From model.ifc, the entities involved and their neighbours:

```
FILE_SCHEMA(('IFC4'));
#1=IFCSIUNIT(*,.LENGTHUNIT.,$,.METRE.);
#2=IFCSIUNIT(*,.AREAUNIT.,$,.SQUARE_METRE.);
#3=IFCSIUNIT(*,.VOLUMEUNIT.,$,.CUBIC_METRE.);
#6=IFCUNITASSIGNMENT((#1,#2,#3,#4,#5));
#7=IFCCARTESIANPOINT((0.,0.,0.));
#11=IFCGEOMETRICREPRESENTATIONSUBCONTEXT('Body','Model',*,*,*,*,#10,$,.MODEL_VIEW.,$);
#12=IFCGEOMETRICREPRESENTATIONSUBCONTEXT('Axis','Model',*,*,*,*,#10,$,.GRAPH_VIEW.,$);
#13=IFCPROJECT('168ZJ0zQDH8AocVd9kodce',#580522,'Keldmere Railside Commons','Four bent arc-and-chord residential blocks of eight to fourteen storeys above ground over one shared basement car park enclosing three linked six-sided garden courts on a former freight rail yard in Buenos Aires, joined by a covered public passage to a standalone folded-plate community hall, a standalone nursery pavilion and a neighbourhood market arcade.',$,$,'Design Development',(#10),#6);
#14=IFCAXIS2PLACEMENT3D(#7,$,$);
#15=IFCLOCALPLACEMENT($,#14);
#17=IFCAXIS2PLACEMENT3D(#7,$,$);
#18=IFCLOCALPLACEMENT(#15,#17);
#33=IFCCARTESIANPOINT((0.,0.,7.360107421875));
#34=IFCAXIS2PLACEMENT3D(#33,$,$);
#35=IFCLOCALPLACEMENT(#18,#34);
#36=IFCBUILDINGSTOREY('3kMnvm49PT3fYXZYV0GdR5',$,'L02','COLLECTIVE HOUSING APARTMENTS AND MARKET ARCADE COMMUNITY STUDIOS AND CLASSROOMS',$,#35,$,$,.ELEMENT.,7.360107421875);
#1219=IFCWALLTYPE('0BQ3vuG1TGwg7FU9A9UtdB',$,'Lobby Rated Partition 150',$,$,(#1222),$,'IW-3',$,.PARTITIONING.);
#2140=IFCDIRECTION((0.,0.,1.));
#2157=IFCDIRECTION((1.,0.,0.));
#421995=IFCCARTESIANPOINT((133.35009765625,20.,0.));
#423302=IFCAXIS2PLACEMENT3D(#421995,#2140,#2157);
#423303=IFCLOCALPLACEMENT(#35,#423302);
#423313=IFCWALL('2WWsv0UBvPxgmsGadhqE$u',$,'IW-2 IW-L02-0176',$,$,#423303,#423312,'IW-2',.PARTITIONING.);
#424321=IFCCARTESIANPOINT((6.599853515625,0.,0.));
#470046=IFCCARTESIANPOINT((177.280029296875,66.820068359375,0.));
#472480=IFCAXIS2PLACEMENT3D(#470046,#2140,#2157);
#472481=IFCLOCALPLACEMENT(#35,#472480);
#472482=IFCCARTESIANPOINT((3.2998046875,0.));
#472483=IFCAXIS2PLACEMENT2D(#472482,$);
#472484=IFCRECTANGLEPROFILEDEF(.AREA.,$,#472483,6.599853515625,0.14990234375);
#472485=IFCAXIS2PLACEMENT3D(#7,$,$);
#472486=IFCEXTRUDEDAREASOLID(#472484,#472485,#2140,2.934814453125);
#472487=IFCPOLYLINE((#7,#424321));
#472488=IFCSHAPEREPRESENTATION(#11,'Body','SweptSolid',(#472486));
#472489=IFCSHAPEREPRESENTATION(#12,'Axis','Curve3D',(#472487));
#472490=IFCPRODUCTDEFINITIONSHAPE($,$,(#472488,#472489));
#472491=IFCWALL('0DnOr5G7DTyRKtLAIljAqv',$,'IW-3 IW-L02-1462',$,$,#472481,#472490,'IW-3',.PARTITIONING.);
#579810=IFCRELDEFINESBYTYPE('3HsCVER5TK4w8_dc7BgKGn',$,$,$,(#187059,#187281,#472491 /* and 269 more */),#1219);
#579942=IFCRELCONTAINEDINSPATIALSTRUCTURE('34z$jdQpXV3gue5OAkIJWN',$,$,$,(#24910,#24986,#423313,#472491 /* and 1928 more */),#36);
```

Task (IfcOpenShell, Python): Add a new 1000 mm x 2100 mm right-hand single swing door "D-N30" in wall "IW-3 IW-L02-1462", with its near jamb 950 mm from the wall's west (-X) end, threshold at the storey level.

```python
import numpy as np
import ifcopenshell
import ifcopenshell.api.feature
import ifcopenshell.api.geometry
import ifcopenshell.api.root
import ifcopenshell.api.spatial
import ifcopenshell.geom
import ifcopenshell.util.element
import ifcopenshell.util.placement
import ifcopenshell.util.representation
import ifcopenshell.util.shape
import ifcopenshell.util.unit

model = ifcopenshell.open("model.ifc")
unit_scale = ifcopenshell.util.unit.calculate_unit_scale(model)
settings = ifcopenshell.geom.settings()


def volume(element):
    """Net volume in cubic metres, openings subtracted."""
    shape = ifcopenshell.geom.create_shape(settings, element)
    return ifcopenshell.util.shape.get_volume(shape.geometry)


wall = model.by_guid("0DnOr5G7DTyRKtLAIljAqv")
storey = ifcopenshell.util.element.get_container(wall, ifc_class="IfcBuildingStorey")
context = ifcopenshell.util.representation.get_context(model, "Model", "Body", "MODEL_VIEW")
before = volume(wall)

width, height, from_end, sill = 1, 2.1, 0.95, 0.0  # metres

# The wall runs along its own X axis, and the end named is its -X end.
wall_shape = ifcopenshell.geom.create_shape(settings, wall)
x, y, z = ifcopenshell.util.shape.get_vertices(wall_shape.geometry).T
start = x.min() + from_end
face, thickness = float(y.min()), float(y.max() - y.min())
wall_matrix = ifcopenshell.util.placement.get_local_placement(wall.ObjectPlacement)
level = ifcopenshell.util.placement.get_local_placement(storey.ObjectPlacement)[2, 3]


def in_wall(x, y):
    """Placement at x, y metres in the wall's axes, at sill height."""
    matrix = wall_matrix.copy()
    matrix[:, 3] = wall_matrix @ np.array([x / unit_scale, y / unit_scale, 0.0, 1.0])
    matrix[2, 3] = level + sill / unit_scale
    return matrix


# Opening: a box that overshoots both wall faces by 50 mm.
opening = ifcopenshell.api.root.create_entity(model, ifc_class="IfcOpeningElement", predefined_type="OPENING")
box = ifcopenshell.api.geometry.add_wall_representation(
    model, context=context, length=width, height=height, thickness=thickness + 0.1
)
ifcopenshell.api.geometry.assign_representation(model, product=opening, representation=box)
ifcopenshell.api.geometry.edit_object_placement(model, product=opening, matrix=in_wall(start, face - 0.05), is_si=False)
ifcopenshell.api.feature.add_feature(model, feature=opening, element=wall)

door = ifcopenshell.api.root.create_entity(model, ifc_class="IfcDoor", name="D-N30", predefined_type="DOOR")
door.OverallWidth, door.OverallHeight = width / unit_scale, height / unit_scale
door.OperationType = "SINGLE_SWING_RIGHT"
body = ifcopenshell.api.geometry.add_door_representation(
    model,
    context=context,
    overall_width=door.OverallWidth,
    overall_height=door.OverallHeight,
    operation_type="SINGLE_SWING_RIGHT",
    lining_properties={"LiningDepth": thickness / unit_scale, "ThresholdDepth": thickness / unit_scale},
)
ifcopenshell.api.geometry.assign_representation(model, product=door, representation=body)
ifcopenshell.api.spatial.assign_container(model, products=[door], relating_structure=storey)
ifcopenshell.api.feature.add_filling(model, opening=opening, element=door)

# The lining spans the wall, so the door starts at the wall face.
ifcopenshell.api.geometry.edit_object_placement(model, product=door, matrix=in_wall(start, face), is_si=False)

after = volume(wall)

print(f"wall volume {before:.3f} -> {after:.3f} m3")

model.write("model_edited.ifc")
```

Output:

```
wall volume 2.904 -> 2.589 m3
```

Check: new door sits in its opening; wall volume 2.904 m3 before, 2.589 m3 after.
